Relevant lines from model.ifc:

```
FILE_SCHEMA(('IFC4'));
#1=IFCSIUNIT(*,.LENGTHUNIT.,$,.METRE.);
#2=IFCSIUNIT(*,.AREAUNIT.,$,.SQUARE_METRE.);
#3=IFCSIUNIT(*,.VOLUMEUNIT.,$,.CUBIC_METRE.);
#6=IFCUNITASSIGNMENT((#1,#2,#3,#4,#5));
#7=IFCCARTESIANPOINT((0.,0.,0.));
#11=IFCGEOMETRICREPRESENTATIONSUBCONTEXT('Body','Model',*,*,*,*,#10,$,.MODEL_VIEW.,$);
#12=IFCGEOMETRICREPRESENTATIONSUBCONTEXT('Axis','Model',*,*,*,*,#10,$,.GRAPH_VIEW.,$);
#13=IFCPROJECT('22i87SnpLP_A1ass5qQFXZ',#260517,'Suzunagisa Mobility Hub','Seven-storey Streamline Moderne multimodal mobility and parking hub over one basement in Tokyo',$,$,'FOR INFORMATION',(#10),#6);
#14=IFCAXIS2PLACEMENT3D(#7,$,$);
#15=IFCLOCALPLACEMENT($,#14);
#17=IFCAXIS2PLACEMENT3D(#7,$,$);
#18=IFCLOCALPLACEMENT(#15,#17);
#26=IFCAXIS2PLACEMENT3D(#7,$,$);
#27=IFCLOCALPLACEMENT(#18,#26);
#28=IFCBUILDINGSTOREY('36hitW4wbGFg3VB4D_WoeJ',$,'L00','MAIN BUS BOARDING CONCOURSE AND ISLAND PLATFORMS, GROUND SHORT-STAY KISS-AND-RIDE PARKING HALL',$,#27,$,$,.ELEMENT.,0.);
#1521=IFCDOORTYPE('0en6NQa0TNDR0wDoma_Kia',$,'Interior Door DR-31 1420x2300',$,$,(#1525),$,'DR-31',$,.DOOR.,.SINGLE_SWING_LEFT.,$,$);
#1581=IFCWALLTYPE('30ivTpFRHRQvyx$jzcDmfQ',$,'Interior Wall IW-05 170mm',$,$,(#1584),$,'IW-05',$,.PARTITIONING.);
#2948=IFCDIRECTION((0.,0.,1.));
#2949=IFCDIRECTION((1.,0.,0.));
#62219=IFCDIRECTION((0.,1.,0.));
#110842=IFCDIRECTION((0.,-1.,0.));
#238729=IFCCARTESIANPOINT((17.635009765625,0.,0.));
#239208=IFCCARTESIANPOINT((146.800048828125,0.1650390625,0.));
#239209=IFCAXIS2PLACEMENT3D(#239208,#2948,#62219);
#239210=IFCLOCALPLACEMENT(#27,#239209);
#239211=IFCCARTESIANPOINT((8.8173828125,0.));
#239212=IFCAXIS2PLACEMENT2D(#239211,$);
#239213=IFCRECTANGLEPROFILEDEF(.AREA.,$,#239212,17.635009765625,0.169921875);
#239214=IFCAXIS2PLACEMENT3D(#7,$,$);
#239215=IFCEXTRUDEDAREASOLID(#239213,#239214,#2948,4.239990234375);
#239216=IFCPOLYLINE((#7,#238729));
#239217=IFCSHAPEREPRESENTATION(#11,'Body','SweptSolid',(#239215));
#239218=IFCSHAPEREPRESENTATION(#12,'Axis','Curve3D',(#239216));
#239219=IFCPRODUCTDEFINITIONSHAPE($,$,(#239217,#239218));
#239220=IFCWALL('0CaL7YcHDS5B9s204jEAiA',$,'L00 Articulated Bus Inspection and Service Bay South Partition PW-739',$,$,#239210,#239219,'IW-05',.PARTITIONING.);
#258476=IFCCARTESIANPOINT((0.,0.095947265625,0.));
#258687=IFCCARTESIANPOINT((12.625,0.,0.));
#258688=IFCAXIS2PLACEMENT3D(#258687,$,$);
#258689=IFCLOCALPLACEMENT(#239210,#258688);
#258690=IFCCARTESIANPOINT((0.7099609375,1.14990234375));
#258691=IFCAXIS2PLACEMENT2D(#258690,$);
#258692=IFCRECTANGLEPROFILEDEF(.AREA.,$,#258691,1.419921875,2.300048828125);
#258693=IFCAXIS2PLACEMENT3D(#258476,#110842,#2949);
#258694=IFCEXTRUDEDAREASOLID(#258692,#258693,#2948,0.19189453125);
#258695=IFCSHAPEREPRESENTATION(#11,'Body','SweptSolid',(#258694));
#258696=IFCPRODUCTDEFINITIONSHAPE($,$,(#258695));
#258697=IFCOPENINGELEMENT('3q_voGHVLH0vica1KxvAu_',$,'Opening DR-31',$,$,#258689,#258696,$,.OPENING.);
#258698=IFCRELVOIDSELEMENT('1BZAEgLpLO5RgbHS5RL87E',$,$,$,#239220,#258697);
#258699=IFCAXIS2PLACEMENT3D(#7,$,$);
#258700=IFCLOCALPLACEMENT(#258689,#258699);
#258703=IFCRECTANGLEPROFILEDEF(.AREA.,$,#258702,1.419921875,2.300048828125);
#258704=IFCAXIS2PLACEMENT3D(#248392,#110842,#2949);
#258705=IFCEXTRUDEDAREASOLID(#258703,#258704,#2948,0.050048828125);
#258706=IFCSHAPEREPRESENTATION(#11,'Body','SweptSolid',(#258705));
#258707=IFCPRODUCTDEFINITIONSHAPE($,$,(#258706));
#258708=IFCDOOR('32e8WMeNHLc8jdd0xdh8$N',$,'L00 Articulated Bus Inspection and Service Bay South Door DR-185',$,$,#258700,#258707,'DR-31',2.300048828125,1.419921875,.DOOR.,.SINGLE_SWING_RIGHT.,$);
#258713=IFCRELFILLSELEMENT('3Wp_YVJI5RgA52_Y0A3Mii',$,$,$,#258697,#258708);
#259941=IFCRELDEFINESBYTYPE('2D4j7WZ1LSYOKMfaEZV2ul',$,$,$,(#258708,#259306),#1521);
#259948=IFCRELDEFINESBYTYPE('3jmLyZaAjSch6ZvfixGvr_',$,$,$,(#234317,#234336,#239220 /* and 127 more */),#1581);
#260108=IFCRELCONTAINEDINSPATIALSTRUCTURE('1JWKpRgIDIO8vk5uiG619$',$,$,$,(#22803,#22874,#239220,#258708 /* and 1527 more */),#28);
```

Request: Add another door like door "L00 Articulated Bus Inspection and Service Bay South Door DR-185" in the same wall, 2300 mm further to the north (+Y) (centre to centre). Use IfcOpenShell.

```python
import ifcopenshell
import ifcopenshell.api.feature
import ifcopenshell.api.geometry
import ifcopenshell.api.root
import ifcopenshell.geom
import ifcopenshell.util.element
import ifcopenshell.util.placement
import ifcopenshell.util.shape

model = ifcopenshell.open("model.ifc")
settings = ifcopenshell.geom.settings()


def volume(element):
    """Net volume in cubic metres, openings subtracted."""
    shape = ifcopenshell.geom.create_shape(settings, element)
    return ifcopenshell.util.shape.get_volume(shape.geometry)


door = model.by_guid("32e8WMeNHLc8jdd0xdh8$N")
opening = door.FillsVoids[0].RelatingOpeningElement
wall = opening.VoidsElements[0].RelatingBuildingElement
before = volume(wall)
shift = ifcopenshell.util.placement.get_local_placement(wall.ObjectPlacement)[:3, 0] * 2.3

# copy_class copies the void relationship, type, container and properties, but no geometry.
new_opening = ifcopenshell.api.root.copy_class(model, product=opening)
new_opening.Representation = ifcopenshell.util.element.copy_deep(
    model, opening.Representation, exclude=["IfcGeometricRepresentationContext", "IfcRepresentationMap"]
)
new_door = ifcopenshell.api.root.copy_class(model, product=door)
new_door.Representation = ifcopenshell.util.element.copy_deep(
    model, door.Representation, exclude=["IfcGeometricRepresentationContext", "IfcRepresentationMap"]
)
new_door.Tag = None
ifcopenshell.api.feature.add_filling(model, opening=new_opening, element=new_door)

for old, new in ((opening, new_opening), (door, new_door)):
    matrix = ifcopenshell.util.placement.get_local_placement(old.ObjectPlacement)
    matrix[:3, 3] += shift
    ifcopenshell.api.geometry.edit_object_placement(model, product=new, matrix=matrix, is_si=False)

after = volume(wall)

print(f"wall volume {before:.3f} -> {after:.3f} m3")

model.write("model_edited.ifc")
```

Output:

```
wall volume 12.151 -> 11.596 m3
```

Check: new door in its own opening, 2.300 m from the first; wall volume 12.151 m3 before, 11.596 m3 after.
